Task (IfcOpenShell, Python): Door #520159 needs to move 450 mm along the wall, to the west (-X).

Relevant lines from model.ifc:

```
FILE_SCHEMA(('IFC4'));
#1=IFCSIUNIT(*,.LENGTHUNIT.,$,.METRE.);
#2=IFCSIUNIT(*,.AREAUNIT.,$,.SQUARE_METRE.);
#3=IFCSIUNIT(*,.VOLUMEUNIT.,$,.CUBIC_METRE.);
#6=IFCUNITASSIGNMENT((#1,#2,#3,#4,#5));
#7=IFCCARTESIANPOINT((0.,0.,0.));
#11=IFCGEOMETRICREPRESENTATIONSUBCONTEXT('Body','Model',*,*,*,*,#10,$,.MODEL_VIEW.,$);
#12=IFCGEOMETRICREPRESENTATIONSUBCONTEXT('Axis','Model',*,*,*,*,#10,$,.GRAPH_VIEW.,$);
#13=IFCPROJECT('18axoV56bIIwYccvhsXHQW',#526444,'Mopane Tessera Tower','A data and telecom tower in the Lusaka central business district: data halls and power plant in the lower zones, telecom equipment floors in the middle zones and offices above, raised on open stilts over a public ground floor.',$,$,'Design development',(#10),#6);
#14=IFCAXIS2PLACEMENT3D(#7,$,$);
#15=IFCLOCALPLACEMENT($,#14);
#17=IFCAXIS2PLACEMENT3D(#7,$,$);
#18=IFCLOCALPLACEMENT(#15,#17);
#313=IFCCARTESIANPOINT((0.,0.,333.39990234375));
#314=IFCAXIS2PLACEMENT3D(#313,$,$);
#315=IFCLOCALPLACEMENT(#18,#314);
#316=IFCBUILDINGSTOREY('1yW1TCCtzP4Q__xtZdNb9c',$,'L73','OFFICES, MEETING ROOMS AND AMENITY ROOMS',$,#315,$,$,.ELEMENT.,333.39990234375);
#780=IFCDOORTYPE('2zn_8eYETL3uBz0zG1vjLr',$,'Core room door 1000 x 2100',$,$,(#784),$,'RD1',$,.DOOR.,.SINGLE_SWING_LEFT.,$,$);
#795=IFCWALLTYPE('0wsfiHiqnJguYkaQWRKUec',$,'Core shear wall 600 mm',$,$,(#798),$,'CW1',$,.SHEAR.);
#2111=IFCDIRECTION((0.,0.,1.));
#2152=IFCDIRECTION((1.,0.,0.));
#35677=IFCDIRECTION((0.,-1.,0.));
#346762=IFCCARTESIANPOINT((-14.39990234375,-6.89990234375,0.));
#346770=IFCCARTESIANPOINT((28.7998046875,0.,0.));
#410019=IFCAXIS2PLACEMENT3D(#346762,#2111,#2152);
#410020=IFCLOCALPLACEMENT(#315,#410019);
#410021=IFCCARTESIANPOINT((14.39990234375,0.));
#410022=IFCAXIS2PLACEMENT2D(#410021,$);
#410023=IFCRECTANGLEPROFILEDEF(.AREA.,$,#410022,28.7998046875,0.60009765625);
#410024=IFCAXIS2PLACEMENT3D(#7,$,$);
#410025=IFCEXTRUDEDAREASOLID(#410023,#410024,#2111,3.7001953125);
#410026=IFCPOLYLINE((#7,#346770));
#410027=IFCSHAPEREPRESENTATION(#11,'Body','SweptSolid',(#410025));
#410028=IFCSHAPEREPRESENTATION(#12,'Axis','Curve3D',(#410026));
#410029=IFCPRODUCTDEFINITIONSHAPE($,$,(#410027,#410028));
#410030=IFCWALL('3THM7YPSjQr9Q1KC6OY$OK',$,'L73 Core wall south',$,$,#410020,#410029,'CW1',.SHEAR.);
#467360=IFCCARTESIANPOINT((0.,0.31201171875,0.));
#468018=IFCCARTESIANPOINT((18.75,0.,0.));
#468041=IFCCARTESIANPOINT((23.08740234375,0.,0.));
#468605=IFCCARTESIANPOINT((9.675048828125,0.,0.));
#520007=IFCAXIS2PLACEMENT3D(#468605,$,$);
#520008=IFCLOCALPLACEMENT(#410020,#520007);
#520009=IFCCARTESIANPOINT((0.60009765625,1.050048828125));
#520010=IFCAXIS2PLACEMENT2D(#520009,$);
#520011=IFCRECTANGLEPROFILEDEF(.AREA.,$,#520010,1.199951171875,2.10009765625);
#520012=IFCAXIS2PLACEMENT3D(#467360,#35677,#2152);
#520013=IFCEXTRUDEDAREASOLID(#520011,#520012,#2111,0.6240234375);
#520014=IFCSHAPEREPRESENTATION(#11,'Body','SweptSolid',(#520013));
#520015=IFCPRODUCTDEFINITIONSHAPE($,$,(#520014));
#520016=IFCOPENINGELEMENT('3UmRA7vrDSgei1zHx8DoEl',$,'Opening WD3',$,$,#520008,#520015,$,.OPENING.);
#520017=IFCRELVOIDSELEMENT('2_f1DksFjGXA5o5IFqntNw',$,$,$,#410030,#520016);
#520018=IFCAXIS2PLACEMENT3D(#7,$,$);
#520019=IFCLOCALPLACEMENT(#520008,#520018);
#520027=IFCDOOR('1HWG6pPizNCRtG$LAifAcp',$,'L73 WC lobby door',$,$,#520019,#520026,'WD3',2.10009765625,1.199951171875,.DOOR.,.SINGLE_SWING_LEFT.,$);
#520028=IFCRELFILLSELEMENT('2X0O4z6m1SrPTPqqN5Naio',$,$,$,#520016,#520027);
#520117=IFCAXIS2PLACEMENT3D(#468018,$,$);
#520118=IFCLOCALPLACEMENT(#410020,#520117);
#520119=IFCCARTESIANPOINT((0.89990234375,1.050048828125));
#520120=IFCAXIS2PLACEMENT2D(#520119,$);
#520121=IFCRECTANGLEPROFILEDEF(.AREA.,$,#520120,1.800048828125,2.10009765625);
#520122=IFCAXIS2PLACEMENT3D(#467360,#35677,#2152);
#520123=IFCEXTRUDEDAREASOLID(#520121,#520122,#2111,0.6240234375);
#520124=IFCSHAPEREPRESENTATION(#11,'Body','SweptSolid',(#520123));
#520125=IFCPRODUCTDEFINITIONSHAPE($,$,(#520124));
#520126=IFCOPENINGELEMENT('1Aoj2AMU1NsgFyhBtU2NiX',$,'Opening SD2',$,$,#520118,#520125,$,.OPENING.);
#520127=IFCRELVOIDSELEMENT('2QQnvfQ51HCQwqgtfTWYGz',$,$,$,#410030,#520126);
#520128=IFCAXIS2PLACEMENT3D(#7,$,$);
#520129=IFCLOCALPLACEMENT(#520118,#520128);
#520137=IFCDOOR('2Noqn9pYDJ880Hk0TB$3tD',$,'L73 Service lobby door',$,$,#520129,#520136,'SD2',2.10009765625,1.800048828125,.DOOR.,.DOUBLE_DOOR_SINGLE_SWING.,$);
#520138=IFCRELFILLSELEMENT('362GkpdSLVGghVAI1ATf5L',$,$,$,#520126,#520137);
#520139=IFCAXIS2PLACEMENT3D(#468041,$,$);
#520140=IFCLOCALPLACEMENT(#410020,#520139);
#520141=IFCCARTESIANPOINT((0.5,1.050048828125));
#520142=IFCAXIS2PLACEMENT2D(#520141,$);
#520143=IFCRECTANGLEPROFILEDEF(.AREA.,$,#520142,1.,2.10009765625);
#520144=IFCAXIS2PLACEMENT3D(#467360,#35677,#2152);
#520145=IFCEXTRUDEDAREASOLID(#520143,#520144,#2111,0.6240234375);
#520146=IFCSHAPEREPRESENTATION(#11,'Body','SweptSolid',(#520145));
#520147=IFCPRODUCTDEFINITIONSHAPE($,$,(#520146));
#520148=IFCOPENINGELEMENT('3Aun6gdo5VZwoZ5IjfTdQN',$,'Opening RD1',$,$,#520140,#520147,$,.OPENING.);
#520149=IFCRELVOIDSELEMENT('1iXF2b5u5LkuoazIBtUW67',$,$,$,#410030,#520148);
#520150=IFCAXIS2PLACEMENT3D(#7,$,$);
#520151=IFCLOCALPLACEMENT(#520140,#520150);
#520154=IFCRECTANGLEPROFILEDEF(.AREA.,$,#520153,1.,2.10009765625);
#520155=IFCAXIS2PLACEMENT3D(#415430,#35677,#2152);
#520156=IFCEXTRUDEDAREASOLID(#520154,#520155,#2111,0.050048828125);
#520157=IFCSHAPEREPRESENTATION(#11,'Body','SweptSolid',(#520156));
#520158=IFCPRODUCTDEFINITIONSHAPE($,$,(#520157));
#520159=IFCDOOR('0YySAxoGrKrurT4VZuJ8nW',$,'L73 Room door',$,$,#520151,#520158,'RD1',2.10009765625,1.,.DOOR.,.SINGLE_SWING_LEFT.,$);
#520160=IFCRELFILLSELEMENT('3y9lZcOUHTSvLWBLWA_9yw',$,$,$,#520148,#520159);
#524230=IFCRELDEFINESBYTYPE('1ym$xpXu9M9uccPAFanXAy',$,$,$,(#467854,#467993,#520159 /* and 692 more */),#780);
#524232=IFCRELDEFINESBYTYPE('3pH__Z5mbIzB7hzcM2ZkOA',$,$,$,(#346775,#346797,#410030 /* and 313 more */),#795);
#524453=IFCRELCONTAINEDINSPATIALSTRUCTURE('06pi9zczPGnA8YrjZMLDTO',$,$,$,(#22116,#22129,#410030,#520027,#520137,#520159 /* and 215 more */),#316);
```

```python
import ifcopenshell
import ifcopenshell.api.geometry
import ifcopenshell.util.placement
import ifcopenshell.util.unit

model = ifcopenshell.open("model.ifc")
unit_scale = ifcopenshell.util.unit.calculate_unit_scale(model)

door = model.by_guid("0YySAxoGrKrurT4VZuJ8nW")
opening = door.FillsVoids[0].RelatingOpeningElement
wall = opening.VoidsElements[0].RelatingBuildingElement

wall_matrix = ifcopenshell.util.placement.get_local_placement(wall.ObjectPlacement)
shift = wall_matrix[:3, 0] * -0.45 / unit_scale
before = ifcopenshell.util.placement.get_local_placement(door.ObjectPlacement)[:3, 3].copy()

# The door is placed relative to its opening, so it follows when the opening moves.
matrix = ifcopenshell.util.placement.get_local_placement(opening.ObjectPlacement)
matrix[:3, 3] += shift
ifcopenshell.api.geometry.edit_object_placement(
    model, product=opening, matrix=matrix, is_si=False, should_transform_children=True
)

after = ifcopenshell.util.placement.get_local_placement(door.ObjectPlacement)[:3, 3]
print("door moved by", (after - before).round(3) + 0.0)

model.write("model_rev.ifc")
```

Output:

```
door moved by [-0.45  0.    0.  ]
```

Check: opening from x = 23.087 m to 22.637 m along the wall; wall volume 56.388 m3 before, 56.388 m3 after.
